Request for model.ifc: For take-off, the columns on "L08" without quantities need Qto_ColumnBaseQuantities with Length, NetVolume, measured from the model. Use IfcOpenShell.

First a look at what the model holds.

```python
import ifcopenshell
import ifcopenshell.util.element
import ifcopenshell.util.unit

model = ifcopenshell.open("model.ifc")
print(model.schema)
for unit_type in ("LENGTHUNIT", "AREAUNIT", "VOLUMEUNIT"):
    print(unit_type, ifcopenshell.util.unit.calculate_unit_scale(model, unit_type))
storey = next(s for s in model.by_type("IfcBuildingStorey") if s.Name == "L08")
columns = [e for e in ifcopenshell.util.element.get_decomposition(storey) if e.is_a("IfcColumn")]
for e in sorted(columns, key=lambda e: e.id()):
    print(e.id(), e.is_a(), e.Name, list(ifcopenshell.util.element.get_psets(e, qtos_only=True)), sep=" | ")
```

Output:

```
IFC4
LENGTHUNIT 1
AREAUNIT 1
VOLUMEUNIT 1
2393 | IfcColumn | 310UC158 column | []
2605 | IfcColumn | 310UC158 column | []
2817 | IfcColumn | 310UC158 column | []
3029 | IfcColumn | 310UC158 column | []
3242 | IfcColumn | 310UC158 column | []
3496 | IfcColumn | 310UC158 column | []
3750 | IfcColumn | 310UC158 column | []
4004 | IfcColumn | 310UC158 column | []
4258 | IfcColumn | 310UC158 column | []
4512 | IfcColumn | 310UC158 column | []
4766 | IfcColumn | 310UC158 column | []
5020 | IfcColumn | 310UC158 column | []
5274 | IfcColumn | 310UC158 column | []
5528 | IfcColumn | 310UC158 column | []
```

```python
import ifcopenshell
import ifcopenshell.api.pset
import ifcopenshell.geom
import ifcopenshell.util.element
import ifcopenshell.util.shape
import ifcopenshell.util.unit

model = ifcopenshell.open("model.ifc")
unit_scale = ifcopenshell.util.unit.calculate_unit_scale(model)
volume_scale = ifcopenshell.util.unit.calculate_unit_scale(model, "VOLUMEUNIT")
settings = ifcopenshell.geom.settings()

storey = next(s for s in model.by_type("IfcBuildingStorey") if s.Name == "L08")
columns = [e for e in ifcopenshell.util.element.get_decomposition(storey) if e.is_a("IfcColumn")]

for e in sorted(columns, key=lambda e: e.id()):
    if ifcopenshell.util.element.get_psets(e, qtos_only=True, should_inherit=False):
        continue
    # Geometry comes back in metres, in the element's own axes.
    shape = ifcopenshell.geom.create_shape(settings, e)
    values = {
        "Length": ifcopenshell.util.shape.get_z(shape.geometry) / unit_scale,
        "NetVolume": ifcopenshell.util.shape.get_volume(shape.geometry) / volume_scale,
    }
    qto = ifcopenshell.api.pset.add_qto(model, product=e, name="Qto_ColumnBaseQuantities")
    ifcopenshell.api.pset.edit_qto(model, qto=qto, properties=values)
    print(e.id(), {k: round(v, 3) for k, v in values.items()})

model.write("model_v2.ifc")
```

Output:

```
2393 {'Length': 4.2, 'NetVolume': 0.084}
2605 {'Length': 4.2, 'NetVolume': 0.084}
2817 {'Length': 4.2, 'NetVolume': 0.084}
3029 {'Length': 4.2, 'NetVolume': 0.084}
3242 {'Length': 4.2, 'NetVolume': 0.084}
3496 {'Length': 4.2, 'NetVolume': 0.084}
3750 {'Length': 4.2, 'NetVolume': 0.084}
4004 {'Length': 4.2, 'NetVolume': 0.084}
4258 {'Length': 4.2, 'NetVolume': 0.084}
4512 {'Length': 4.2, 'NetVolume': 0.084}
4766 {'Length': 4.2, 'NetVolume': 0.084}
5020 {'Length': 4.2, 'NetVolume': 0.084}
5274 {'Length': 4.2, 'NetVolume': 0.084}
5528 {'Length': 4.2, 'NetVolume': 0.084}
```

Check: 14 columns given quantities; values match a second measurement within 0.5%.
